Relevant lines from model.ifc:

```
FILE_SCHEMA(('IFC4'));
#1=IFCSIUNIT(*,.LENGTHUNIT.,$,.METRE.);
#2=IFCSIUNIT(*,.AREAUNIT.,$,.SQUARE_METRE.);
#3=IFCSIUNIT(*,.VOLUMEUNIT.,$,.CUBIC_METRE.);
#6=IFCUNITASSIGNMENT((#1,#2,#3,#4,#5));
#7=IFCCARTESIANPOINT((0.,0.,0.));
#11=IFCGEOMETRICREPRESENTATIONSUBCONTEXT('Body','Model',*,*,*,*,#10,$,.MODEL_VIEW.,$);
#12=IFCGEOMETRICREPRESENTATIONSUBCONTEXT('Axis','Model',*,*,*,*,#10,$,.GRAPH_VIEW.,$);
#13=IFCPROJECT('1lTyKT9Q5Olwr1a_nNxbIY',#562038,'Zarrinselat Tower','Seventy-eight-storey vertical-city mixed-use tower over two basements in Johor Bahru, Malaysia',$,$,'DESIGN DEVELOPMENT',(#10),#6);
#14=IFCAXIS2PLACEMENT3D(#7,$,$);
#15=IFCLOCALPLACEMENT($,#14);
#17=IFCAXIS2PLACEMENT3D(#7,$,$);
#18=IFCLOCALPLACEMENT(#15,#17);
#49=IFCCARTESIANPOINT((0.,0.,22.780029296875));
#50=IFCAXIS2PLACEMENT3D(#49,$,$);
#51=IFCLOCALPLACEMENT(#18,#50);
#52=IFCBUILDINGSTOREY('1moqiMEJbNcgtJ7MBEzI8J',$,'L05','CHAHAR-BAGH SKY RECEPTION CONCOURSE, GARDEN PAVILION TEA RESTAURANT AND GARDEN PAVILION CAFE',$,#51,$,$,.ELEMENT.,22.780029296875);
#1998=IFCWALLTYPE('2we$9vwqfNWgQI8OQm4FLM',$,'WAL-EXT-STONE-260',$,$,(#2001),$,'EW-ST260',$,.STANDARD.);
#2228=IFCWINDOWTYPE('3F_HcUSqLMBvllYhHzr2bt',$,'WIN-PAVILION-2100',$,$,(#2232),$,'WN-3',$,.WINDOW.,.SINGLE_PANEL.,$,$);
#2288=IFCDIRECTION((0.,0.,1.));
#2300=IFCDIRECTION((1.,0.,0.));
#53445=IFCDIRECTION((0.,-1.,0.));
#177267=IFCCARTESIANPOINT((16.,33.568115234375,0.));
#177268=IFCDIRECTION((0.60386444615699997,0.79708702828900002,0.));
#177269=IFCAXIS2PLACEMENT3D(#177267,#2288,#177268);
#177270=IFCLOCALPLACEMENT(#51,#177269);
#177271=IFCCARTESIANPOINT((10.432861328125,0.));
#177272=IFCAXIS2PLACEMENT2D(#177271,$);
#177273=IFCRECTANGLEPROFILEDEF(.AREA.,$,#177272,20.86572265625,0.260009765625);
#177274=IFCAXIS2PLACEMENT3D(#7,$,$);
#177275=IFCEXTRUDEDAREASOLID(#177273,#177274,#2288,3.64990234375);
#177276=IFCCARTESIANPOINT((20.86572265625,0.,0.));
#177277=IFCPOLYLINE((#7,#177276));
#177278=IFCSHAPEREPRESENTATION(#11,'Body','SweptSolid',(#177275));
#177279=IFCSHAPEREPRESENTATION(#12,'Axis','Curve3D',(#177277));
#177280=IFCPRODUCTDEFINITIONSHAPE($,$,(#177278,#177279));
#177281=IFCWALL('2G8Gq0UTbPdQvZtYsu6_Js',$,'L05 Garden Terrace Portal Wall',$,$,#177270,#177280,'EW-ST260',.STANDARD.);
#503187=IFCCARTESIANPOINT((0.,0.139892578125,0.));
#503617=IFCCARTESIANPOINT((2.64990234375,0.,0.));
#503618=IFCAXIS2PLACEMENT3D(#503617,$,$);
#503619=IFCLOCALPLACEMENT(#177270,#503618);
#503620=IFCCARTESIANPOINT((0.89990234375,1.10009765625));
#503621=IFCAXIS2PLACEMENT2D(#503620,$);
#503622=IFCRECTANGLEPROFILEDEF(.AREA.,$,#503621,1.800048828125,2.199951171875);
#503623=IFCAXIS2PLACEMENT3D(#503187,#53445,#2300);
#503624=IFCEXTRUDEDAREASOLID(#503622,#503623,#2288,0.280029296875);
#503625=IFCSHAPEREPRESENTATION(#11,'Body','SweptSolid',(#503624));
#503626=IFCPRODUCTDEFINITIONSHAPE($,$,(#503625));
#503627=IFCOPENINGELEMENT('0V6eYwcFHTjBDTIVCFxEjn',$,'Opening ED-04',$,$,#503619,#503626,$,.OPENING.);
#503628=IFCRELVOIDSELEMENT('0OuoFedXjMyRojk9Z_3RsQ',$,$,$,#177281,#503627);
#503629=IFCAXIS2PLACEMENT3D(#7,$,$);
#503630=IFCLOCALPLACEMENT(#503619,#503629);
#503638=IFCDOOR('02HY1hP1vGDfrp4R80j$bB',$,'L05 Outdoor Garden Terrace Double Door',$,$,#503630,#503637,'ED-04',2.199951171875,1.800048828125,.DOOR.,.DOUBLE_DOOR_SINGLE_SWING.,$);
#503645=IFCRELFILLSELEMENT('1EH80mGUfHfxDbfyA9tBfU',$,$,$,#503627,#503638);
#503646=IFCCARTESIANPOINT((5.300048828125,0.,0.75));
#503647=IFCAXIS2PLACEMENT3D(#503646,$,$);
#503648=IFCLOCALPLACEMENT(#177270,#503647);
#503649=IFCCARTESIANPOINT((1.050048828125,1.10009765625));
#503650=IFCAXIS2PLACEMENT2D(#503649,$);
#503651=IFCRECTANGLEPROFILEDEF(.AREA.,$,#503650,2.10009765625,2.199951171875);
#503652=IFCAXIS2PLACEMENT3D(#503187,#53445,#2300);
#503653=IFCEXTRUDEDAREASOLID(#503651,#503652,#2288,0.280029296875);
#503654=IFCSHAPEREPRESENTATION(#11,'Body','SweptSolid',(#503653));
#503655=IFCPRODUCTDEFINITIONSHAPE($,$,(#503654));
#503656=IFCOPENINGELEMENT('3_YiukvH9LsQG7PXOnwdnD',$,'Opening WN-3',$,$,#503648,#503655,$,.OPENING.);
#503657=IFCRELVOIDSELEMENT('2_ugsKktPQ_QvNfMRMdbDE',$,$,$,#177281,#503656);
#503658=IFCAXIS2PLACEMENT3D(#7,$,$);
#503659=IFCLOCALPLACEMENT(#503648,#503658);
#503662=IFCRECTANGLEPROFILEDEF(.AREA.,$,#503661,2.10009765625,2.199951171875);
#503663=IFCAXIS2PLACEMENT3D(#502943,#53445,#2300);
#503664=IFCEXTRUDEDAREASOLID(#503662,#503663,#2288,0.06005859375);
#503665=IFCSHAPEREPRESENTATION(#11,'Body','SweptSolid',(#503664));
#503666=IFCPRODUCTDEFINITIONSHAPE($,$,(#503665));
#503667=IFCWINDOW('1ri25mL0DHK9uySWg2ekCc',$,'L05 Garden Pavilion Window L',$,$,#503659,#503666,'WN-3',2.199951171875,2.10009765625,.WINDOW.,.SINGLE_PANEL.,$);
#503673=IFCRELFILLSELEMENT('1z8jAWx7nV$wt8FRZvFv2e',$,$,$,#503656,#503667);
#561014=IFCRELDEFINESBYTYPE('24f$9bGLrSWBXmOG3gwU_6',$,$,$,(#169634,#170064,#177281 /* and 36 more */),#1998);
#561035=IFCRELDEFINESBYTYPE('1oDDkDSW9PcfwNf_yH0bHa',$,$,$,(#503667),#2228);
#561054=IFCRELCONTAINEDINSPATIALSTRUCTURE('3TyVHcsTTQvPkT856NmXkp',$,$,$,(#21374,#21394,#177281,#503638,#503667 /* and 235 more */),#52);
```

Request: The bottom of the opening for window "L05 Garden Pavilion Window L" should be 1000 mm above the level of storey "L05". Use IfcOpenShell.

```python
import numpy as np
import ifcopenshell
import ifcopenshell.api.geometry
import ifcopenshell.geom
import ifcopenshell.util.element
import ifcopenshell.util.placement
import ifcopenshell.util.shape
import ifcopenshell.util.unit

model = ifcopenshell.open("model.ifc")
unit_scale = ifcopenshell.util.unit.calculate_unit_scale(model)

window = model.by_guid("1ri25mL0DHK9uySWg2ekCc")
opening = window.FillsVoids[0].RelatingOpeningElement
storey = ifcopenshell.util.element.get_container(window, ifc_class="IfcBuildingStorey")
level = ifcopenshell.util.placement.get_local_placement(storey.ObjectPlacement)[2, 3]

# The opening's origin need not be at the sill, so measure its lowest point.
shape = ifcopenshell.geom.create_shape(ifcopenshell.geom.settings(), opening)
bottom = ifcopenshell.util.shape.get_shape_bottom_elevation(shape, shape.geometry) / unit_scale
dz = level + 1 / unit_scale - bottom

shift = np.array([0.0, 0.0, dz])
# The window is placed relative to its opening, so it follows when the opening moves.
matrix = ifcopenshell.util.placement.get_local_placement(opening.ObjectPlacement)
matrix[:3, 3] += shift
ifcopenshell.api.geometry.edit_object_placement(
    model, product=opening, matrix=matrix, is_si=False, should_transform_children=True
)

print(f"moved by {dz * unit_scale:+.3f} m")

model.write("model_updated.ifc")
```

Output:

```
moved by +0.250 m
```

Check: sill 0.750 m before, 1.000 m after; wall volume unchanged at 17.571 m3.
